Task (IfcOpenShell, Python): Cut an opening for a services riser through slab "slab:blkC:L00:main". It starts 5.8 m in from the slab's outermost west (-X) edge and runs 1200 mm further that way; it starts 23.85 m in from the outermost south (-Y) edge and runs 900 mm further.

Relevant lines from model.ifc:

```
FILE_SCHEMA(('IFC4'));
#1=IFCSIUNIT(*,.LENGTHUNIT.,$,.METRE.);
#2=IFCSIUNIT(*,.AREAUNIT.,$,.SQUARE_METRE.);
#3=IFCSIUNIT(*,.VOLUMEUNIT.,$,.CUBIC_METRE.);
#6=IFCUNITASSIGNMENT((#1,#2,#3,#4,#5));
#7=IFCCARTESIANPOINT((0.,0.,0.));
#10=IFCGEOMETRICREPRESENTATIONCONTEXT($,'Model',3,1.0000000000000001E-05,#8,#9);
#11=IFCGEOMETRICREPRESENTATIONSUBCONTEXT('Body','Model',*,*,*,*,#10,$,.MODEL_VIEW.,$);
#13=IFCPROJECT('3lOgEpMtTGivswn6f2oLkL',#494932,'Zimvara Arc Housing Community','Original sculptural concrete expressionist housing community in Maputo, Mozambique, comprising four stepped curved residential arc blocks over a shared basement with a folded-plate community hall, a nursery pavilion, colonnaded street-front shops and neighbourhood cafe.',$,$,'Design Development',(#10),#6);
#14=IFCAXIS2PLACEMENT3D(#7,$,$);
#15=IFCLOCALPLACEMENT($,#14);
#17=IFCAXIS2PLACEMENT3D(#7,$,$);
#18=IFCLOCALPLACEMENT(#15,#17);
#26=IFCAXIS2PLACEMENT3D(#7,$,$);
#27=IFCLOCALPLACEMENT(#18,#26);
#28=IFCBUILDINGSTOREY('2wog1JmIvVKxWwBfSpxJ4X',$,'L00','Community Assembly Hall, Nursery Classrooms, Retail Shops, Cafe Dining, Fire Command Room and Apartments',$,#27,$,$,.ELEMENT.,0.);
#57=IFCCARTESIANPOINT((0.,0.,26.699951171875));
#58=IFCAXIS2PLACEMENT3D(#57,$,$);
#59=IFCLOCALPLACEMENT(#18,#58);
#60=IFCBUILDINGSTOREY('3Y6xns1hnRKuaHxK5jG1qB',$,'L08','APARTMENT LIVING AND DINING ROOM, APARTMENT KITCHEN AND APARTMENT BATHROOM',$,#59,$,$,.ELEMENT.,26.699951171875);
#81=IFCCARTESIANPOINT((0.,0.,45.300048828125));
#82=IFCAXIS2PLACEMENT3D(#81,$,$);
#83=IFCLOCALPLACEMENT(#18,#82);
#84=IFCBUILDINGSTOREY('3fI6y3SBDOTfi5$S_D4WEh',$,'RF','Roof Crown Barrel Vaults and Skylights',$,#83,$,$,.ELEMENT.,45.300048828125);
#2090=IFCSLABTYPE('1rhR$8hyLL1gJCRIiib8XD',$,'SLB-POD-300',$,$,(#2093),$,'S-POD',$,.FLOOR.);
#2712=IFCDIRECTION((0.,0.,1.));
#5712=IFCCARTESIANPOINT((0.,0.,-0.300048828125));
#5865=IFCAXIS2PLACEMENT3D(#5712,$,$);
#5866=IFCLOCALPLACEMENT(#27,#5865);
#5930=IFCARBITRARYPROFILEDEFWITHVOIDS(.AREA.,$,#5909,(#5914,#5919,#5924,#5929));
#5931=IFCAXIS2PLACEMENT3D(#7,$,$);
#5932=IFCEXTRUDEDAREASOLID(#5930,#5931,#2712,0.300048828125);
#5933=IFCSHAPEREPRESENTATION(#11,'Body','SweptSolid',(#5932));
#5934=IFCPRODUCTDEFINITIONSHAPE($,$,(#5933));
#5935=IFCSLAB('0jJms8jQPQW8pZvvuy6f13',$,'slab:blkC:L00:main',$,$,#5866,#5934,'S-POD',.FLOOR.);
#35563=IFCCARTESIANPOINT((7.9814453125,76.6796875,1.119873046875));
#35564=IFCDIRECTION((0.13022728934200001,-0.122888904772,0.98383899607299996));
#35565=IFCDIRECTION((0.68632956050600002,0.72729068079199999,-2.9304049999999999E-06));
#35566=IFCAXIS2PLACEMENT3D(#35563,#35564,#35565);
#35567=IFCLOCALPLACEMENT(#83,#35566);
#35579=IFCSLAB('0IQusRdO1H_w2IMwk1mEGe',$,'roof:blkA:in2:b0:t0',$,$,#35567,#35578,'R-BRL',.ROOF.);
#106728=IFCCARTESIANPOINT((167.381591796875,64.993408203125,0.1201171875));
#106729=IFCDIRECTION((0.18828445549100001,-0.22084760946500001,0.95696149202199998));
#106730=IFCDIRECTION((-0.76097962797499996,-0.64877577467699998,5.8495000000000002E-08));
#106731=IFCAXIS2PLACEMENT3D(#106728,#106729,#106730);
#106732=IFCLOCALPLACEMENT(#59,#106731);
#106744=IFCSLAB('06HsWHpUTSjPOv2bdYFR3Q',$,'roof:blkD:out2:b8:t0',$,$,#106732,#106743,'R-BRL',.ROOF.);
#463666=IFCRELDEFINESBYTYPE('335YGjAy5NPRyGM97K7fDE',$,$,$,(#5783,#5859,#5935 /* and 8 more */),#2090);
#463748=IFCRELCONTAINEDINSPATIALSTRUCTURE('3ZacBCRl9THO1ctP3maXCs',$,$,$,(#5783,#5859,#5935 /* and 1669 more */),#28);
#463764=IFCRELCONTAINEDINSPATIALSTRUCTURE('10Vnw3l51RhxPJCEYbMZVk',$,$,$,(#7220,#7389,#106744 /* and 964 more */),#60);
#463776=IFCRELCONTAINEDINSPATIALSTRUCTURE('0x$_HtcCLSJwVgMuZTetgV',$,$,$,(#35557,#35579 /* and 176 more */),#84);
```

```python
import numpy as np
import ifcopenshell
import ifcopenshell.api.feature
import ifcopenshell.api.geometry
import ifcopenshell.api.root
import ifcopenshell.geom
import ifcopenshell.util.placement
import ifcopenshell.util.representation
import ifcopenshell.util.shape
import ifcopenshell.util.unit

model = ifcopenshell.open("model.ifc")
unit_scale = ifcopenshell.util.unit.calculate_unit_scale(model)
settings = ifcopenshell.geom.settings()


def volume(element):
    """Net volume in cubic metres, openings subtracted."""
    shape = ifcopenshell.geom.create_shape(settings, element)
    return ifcopenshell.util.shape.get_volume(shape.geometry)


slab = model.by_guid("0jJms8jQPQW8pZvvuy6f13")
before = volume(slab)

# Extent in the slab's own axes, in metres. The edges named are its -X and -Y sides.
slab_shape = ifcopenshell.geom.create_shape(settings, slab)
vertices = ifcopenshell.util.shape.get_vertices(slab_shape.geometry)
x_min, y_min, bottom = vertices.min(axis=0)
top = vertices[:, 2].max()

opening = ifcopenshell.api.root.create_entity(model, ifc_class="IfcOpeningElement", name="Services riser opening", predefined_type="OPENING")
context = ifcopenshell.util.representation.get_context(model, "Model", "Body", "MODEL_VIEW")
width, depth = 1.2, 0.9
outline = [(0.0, 0.0), (width, 0.0), (width, depth), (0.0, depth), (0.0, 0.0)]
# Overshoot both faces by 50 mm so the cut is clean.
shape = ifcopenshell.api.geometry.add_slab_representation(
    model, context=context, depth=top - bottom + 0.1, polyline=outline
)
ifcopenshell.api.geometry.assign_representation(model, product=opening, representation=shape)

matrix = ifcopenshell.util.placement.get_local_placement(slab.ObjectPlacement)
matrix[:, 3] = matrix @ np.append(np.array([x_min + 5.8, y_min + 23.85, bottom - 0.05]) / unit_scale, 1.0)
ifcopenshell.api.geometry.edit_object_placement(model, product=opening, matrix=matrix, is_si=False)
ifcopenshell.api.feature.add_feature(model, feature=opening, element=slab)

after = volume(slab)

print(f"slab volume {before:.3f} -> {after:.3f} m3")

model.write("model_v2.ifc")
```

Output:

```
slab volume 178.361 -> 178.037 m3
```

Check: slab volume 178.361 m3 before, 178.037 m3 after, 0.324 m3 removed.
